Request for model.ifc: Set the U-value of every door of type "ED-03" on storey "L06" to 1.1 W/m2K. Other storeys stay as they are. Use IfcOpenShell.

First a look at what the model holds.

```python
import ifcopenshell
import ifcopenshell.util.element

model = ifcopenshell.open("model.ifc")
print(model.schema)
storey = next(s for s in model.by_type("IfcBuildingStorey") if s.Name == "L06")
doors = [e for e in ifcopenshell.util.element.get_decomposition(storey) if e.is_a("IfcDoor")]
seen = {}
for e in doors:
    element_type = ifcopenshell.util.element.get_type(e)
    key = (element_type.Name if element_type != e and element_type else None, ifcopenshell.util.element.get_pset(e, "Pset_DoorCommon", "ThermalTransmittance"))
    seen[key] = seen.get(key, 0) + 1
for (name, value), count in sorted(seen.items(), key=str):
    print(count, "x", name, "|", value)
```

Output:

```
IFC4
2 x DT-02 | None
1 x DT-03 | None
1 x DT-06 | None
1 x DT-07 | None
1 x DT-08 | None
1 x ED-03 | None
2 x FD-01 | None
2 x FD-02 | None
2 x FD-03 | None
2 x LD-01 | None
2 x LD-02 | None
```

```python
import ifcopenshell
import ifcopenshell.api.pset
import ifcopenshell.util.element

model = ifcopenshell.open("model.ifc")

storey = next(s for s in model.by_type("IfcBuildingStorey") if s.Name == "L06")
doors = [e for e in ifcopenshell.util.element.get_decomposition(storey) if e.is_a("IfcDoor")]

count = 0
for e in doors:
    element_type = ifcopenshell.util.element.get_type(e)
    if element_type in (None, e) or element_type.Name != "ED-03":
        continue
    # add_pset returns the element's existing set when there is one.
    pset = ifcopenshell.api.pset.add_pset(model, product=e, name="Pset_DoorCommon")
    ifcopenshell.api.pset.edit_pset(model, pset=pset, properties={"ThermalTransmittance": 1.1})
    count += 1

print(count, "doors updated")

model.write("model_v2.ifc")
```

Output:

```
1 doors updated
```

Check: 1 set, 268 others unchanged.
